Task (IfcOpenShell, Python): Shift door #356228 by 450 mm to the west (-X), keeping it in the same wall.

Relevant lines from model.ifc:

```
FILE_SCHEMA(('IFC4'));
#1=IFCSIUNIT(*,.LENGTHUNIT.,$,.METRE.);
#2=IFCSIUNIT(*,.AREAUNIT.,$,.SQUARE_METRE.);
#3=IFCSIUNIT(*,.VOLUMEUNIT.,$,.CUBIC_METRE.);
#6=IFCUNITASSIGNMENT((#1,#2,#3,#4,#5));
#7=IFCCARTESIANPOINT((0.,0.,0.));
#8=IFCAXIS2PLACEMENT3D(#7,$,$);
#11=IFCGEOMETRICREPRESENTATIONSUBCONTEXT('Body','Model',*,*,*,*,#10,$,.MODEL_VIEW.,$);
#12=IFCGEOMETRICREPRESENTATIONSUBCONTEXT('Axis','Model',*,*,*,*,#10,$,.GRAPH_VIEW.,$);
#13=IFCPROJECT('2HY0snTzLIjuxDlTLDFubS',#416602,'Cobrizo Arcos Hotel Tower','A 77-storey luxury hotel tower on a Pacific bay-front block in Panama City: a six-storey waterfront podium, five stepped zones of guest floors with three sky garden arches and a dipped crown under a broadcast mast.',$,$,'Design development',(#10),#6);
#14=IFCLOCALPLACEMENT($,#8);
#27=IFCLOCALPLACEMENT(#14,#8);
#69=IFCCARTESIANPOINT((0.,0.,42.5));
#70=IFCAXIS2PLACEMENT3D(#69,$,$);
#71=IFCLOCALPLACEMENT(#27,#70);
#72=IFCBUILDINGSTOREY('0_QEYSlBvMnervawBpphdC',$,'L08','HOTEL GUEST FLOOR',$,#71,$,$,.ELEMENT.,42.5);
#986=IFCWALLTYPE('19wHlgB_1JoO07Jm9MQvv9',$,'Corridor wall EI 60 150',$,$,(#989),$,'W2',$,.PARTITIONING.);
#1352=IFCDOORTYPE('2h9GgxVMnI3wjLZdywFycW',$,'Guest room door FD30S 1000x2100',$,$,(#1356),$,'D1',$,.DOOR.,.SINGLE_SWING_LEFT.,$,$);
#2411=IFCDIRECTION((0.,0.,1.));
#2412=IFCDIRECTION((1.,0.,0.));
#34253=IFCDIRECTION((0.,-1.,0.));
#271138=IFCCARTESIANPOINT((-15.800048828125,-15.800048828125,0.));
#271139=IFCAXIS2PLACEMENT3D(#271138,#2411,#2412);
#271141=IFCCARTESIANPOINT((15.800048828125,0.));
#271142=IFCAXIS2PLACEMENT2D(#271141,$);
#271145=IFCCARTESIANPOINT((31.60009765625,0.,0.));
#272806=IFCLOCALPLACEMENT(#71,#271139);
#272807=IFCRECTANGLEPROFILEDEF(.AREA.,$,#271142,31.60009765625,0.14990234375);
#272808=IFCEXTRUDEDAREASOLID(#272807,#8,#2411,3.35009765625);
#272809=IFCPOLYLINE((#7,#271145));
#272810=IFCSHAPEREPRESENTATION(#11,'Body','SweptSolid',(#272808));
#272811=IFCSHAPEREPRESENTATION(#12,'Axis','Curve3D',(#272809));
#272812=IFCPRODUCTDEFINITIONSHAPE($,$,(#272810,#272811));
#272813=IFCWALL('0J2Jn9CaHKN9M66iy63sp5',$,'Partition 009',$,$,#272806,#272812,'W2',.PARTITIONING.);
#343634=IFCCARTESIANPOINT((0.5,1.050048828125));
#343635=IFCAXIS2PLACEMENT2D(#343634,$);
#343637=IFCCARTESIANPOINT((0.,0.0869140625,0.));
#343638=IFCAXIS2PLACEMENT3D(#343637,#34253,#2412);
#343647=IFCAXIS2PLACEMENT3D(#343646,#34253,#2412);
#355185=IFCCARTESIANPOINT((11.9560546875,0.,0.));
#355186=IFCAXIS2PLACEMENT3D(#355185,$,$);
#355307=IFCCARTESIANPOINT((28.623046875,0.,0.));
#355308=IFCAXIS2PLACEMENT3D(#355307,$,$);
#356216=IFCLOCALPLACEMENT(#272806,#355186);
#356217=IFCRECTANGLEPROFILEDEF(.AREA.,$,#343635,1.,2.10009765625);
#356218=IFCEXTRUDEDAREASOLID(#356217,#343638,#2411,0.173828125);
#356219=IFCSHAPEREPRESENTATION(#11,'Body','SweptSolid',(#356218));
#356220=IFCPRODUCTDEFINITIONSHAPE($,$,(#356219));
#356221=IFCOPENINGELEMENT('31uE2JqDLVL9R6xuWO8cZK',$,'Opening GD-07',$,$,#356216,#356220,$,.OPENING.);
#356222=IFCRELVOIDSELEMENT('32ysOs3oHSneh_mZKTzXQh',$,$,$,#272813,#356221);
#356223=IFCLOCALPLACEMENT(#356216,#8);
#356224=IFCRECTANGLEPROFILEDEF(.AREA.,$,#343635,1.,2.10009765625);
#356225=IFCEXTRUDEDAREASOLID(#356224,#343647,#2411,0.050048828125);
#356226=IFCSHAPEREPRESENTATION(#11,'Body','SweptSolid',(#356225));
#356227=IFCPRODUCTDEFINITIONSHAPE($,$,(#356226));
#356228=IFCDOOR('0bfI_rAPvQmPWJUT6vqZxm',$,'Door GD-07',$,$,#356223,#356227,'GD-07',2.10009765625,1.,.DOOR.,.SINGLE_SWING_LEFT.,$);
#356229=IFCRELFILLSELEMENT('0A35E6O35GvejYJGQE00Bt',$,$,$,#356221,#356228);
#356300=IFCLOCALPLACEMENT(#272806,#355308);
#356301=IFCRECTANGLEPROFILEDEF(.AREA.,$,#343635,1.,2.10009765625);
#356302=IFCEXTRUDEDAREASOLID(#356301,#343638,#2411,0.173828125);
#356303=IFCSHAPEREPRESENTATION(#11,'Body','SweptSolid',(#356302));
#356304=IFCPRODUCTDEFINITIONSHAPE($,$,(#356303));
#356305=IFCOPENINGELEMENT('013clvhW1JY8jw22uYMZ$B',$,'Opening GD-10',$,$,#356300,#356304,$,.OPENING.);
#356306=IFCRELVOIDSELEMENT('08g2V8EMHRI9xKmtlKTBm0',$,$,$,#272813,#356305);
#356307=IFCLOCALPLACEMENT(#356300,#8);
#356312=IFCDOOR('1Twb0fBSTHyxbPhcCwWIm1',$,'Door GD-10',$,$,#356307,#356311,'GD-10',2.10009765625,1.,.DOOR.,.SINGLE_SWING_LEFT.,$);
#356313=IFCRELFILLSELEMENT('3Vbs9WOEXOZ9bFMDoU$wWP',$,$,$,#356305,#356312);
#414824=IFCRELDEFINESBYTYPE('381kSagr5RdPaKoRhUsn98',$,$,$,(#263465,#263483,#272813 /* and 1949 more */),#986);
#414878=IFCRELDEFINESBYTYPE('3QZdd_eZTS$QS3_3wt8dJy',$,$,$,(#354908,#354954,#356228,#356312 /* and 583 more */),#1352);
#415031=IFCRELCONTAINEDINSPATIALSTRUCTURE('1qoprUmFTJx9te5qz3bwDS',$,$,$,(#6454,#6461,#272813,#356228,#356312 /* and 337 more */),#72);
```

```python
import ifcopenshell
import ifcopenshell.api.geometry
import ifcopenshell.util.placement
import ifcopenshell.util.unit

model = ifcopenshell.open("model.ifc")
unit_scale = ifcopenshell.util.unit.calculate_unit_scale(model)

door = model.by_id(356228)
opening = door.FillsVoids[0].RelatingOpeningElement
wall = opening.VoidsElements[0].RelatingBuildingElement

wall_matrix = ifcopenshell.util.placement.get_local_placement(wall.ObjectPlacement)
shift = wall_matrix[:3, 0] * -0.45 / unit_scale
before = ifcopenshell.util.placement.get_local_placement(door.ObjectPlacement)[:3, 3].copy()

# The door is placed relative to its opening, so it follows when the opening moves.
matrix = ifcopenshell.util.placement.get_local_placement(opening.ObjectPlacement)
matrix[:3, 3] += shift
ifcopenshell.api.geometry.edit_object_placement(
    model, product=opening, matrix=matrix, is_si=False, should_transform_children=True
)

after = ifcopenshell.util.placement.get_local_placement(door.ObjectPlacement)[:3, 3]
print("door moved by", (after - before).round(3) + 0.0)

model.write("model_updated.ifc")
```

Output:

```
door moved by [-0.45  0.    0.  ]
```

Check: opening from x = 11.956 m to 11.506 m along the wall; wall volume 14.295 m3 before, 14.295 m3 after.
